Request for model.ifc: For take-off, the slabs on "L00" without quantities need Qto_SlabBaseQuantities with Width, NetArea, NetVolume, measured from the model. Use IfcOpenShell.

First a look at what the model holds.

```python
import ifcopenshell
import ifcopenshell.util.element
import ifcopenshell.util.unit

model = ifcopenshell.open("model.ifc")
print(model.schema)
for unit_type in ("LENGTHUNIT", "AREAUNIT", "VOLUMEUNIT"):
    print(unit_type, ifcopenshell.util.unit.calculate_unit_scale(model, unit_type))
storey = next(s for s in model.by_type("IfcBuildingStorey") if s.Name == "L00")
slabs = [e for e in ifcopenshell.util.element.get_decomposition(storey) if e.is_a("IfcSlab")]
for e in sorted(slabs, key=lambda e: e.id()):
    print(e.id(), e.is_a(), e.Name, list(ifcopenshell.util.element.get_psets(e, qtos_only=True)), sep=" | ")
```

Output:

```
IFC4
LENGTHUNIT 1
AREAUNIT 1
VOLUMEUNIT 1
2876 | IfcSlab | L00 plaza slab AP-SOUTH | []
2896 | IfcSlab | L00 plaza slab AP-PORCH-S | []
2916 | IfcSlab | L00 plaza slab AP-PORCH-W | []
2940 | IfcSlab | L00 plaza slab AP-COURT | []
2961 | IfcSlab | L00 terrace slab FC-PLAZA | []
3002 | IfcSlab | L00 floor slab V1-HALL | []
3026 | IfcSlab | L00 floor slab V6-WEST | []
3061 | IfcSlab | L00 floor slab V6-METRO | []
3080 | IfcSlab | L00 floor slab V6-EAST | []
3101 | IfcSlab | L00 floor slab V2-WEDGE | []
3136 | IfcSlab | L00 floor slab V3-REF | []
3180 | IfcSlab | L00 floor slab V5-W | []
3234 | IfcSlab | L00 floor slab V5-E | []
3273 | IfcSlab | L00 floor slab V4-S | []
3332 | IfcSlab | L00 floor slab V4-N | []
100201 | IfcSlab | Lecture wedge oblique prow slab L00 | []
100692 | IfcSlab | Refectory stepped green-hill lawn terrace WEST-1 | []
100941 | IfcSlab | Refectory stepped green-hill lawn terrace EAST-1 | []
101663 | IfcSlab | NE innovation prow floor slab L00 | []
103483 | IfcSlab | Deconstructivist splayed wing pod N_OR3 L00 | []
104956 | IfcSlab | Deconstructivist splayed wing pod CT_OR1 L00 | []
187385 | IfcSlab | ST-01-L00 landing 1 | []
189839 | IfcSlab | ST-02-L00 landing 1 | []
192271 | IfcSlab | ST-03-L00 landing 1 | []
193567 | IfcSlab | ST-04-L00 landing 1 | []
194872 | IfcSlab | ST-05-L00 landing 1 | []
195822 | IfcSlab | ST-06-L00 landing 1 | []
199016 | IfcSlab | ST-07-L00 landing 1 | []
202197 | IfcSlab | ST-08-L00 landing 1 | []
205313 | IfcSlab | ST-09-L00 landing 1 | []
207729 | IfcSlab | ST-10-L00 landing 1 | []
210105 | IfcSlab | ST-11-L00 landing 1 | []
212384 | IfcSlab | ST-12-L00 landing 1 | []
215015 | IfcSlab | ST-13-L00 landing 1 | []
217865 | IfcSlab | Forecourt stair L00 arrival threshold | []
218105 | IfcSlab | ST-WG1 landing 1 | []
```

```python
import ifcopenshell
import ifcopenshell.api.pset
import ifcopenshell.geom
import ifcopenshell.util.element
import ifcopenshell.util.shape
import ifcopenshell.util.unit

model = ifcopenshell.open("model.ifc")
unit_scale = ifcopenshell.util.unit.calculate_unit_scale(model)
area_scale = ifcopenshell.util.unit.calculate_unit_scale(model, "AREAUNIT")
volume_scale = ifcopenshell.util.unit.calculate_unit_scale(model, "VOLUMEUNIT")
settings = ifcopenshell.geom.settings()

storey = next(s for s in model.by_type("IfcBuildingStorey") if s.Name == "L00")
slabs = [e for e in ifcopenshell.util.element.get_decomposition(storey) if e.is_a("IfcSlab")]

for e in sorted(slabs, key=lambda e: e.id()):
    if ifcopenshell.util.element.get_psets(e, qtos_only=True, should_inherit=False):
        continue
    # Geometry comes back in metres, in the element's own axes.
    shape = ifcopenshell.geom.create_shape(settings, e)
    values = {
        "Width": ifcopenshell.util.shape.get_z(shape.geometry) / unit_scale,
        "NetArea": ifcopenshell.util.shape.get_footprint_area(shape.geometry) / area_scale,
        "NetVolume": ifcopenshell.util.shape.get_volume(shape.geometry) / volume_scale,
    }
    qto = ifcopenshell.api.pset.add_qto(model, product=e, name="Qto_SlabBaseQuantities")
    ifcopenshell.api.pset.edit_qto(model, qto=qto, properties=values)
    print(e.id(), {k: round(v, 3) for k, v in values.items()})

model.write("model_updated.ifc")
```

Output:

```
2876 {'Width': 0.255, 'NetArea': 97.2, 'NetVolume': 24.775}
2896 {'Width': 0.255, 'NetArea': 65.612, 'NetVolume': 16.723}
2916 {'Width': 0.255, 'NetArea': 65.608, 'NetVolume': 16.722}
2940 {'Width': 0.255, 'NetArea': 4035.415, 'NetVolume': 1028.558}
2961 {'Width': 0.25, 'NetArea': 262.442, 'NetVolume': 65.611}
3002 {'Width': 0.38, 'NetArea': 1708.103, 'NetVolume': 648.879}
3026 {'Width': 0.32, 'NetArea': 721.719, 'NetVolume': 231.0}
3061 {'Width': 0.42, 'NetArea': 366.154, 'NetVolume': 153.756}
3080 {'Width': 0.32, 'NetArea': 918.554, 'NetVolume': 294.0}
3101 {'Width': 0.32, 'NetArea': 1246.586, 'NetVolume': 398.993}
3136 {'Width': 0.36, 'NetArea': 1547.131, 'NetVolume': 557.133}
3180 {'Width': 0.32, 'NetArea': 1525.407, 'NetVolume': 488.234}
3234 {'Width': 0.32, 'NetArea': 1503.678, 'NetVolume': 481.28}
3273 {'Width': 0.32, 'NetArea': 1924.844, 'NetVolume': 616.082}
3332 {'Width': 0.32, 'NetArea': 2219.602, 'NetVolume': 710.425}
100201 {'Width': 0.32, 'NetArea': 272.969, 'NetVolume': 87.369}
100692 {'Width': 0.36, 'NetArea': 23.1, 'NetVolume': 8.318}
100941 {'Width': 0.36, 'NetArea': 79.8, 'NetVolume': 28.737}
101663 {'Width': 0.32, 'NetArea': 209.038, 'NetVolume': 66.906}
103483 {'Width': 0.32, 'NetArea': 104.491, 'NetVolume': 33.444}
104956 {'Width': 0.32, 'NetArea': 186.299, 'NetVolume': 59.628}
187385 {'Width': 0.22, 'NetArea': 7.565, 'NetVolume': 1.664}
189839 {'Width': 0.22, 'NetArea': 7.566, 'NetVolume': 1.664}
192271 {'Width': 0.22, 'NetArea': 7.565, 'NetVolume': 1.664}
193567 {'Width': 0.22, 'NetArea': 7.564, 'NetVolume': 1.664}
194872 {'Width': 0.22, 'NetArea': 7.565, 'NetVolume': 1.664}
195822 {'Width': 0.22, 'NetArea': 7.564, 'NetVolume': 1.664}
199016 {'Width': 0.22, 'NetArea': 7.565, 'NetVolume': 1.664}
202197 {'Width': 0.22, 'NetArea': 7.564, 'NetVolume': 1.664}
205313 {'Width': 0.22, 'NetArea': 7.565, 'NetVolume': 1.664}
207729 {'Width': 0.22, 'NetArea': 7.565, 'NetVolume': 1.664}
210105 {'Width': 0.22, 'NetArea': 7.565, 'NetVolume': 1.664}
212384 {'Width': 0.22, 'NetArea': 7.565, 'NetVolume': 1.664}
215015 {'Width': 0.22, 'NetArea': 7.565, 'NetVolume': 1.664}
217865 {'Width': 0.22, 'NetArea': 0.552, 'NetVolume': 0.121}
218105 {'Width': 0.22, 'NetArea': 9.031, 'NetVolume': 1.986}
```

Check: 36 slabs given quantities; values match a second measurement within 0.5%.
